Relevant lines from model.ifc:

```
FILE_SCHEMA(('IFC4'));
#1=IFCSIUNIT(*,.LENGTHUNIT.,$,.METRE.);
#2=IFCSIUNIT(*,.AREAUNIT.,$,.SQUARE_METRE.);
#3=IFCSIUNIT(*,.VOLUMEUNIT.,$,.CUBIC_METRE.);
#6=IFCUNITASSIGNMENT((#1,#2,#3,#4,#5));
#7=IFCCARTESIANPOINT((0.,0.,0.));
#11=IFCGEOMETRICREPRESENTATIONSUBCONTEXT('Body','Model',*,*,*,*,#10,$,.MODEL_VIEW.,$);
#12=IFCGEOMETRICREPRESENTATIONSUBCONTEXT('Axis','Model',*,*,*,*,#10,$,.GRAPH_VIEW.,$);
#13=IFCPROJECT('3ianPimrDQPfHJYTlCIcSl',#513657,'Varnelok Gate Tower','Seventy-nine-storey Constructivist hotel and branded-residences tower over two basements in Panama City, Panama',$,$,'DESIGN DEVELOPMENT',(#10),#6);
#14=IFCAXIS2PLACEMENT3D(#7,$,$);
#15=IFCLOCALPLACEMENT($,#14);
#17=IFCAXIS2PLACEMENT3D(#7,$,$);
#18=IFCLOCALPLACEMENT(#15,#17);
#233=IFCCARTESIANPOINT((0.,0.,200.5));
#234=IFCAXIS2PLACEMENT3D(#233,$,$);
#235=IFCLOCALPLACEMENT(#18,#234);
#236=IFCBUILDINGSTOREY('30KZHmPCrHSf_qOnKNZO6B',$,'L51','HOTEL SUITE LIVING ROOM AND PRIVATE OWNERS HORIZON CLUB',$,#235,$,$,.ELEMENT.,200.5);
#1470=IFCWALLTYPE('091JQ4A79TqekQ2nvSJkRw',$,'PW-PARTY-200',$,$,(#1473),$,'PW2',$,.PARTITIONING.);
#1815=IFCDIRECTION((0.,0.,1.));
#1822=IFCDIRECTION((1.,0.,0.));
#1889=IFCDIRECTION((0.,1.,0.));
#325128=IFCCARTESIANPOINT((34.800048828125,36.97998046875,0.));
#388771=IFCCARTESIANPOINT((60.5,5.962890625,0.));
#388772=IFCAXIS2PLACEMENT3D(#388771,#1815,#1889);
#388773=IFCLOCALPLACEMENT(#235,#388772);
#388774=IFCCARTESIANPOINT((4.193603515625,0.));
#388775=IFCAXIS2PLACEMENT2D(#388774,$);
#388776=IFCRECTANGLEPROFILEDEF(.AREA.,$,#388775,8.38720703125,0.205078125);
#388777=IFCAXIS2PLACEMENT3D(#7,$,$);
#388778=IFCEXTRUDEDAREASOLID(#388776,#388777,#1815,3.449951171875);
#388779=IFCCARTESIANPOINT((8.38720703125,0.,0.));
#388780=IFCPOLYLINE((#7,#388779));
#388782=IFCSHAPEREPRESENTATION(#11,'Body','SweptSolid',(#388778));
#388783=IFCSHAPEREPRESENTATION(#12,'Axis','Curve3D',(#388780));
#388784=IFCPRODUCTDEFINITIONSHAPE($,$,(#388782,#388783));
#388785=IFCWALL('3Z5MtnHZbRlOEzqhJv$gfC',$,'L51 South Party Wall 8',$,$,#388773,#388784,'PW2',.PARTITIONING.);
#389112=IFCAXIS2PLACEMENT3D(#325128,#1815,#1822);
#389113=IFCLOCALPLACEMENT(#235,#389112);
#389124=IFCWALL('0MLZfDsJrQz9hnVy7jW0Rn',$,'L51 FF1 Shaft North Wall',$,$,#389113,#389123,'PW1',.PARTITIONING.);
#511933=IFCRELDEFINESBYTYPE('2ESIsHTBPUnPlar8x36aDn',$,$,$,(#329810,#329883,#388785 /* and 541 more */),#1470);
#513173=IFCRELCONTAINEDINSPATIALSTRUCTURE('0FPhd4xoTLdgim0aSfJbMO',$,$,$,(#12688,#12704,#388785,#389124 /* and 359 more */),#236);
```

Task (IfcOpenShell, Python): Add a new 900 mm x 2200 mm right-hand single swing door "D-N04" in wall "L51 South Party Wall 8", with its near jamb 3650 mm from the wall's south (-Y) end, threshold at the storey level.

```python
import numpy as np
import ifcopenshell
import ifcopenshell.api.feature
import ifcopenshell.api.geometry
import ifcopenshell.api.root
import ifcopenshell.api.spatial
import ifcopenshell.geom
import ifcopenshell.util.element
import ifcopenshell.util.placement
import ifcopenshell.util.representation
import ifcopenshell.util.shape
import ifcopenshell.util.unit

model = ifcopenshell.open("model.ifc")
unit_scale = ifcopenshell.util.unit.calculate_unit_scale(model)
settings = ifcopenshell.geom.settings()


def volume(element):
    """Net volume in cubic metres, openings subtracted."""
    shape = ifcopenshell.geom.create_shape(settings, element)
    return ifcopenshell.util.shape.get_volume(shape.geometry)


wall = model.by_id(388785)
storey = ifcopenshell.util.element.get_container(wall, ifc_class="IfcBuildingStorey")
context = ifcopenshell.util.representation.get_context(model, "Model", "Body", "MODEL_VIEW")
before = volume(wall)

width, height, from_end, sill = 0.9, 2.2, 3.65, 0.0  # metres

# The wall runs along its own X axis, and the end named is its -X end.
wall_shape = ifcopenshell.geom.create_shape(settings, wall)
x, y, z = ifcopenshell.util.shape.get_vertices(wall_shape.geometry).T
start = x.min() + from_end
face, thickness = float(y.min()), float(y.max() - y.min())
wall_matrix = ifcopenshell.util.placement.get_local_placement(wall.ObjectPlacement)
level = ifcopenshell.util.placement.get_local_placement(storey.ObjectPlacement)[2, 3]


def in_wall(x, y):
    """Placement at x, y metres in the wall's axes, at sill height."""
    matrix = wall_matrix.copy()
    matrix[:, 3] = wall_matrix @ np.array([x / unit_scale, y / unit_scale, 0.0, 1.0])
    matrix[2, 3] = level + sill / unit_scale
    return matrix


# Opening: a box that overshoots both wall faces by 50 mm.
opening = ifcopenshell.api.root.create_entity(model, ifc_class="IfcOpeningElement", predefined_type="OPENING")
box = ifcopenshell.api.geometry.add_wall_representation(
    model, context=context, length=width, height=height, thickness=thickness + 0.1
)
ifcopenshell.api.geometry.assign_representation(model, product=opening, representation=box)
ifcopenshell.api.geometry.edit_object_placement(model, product=opening, matrix=in_wall(start, face - 0.05), is_si=False)
ifcopenshell.api.feature.add_feature(model, feature=opening, element=wall)

door = ifcopenshell.api.root.create_entity(model, ifc_class="IfcDoor", name="D-N04", predefined_type="DOOR")
door.OverallWidth, door.OverallHeight = width / unit_scale, height / unit_scale
door.OperationType = "SINGLE_SWING_RIGHT"
body = ifcopenshell.api.geometry.add_door_representation(
    model,
    context=context,
    overall_width=door.OverallWidth,
    overall_height=door.OverallHeight,
    operation_type="SINGLE_SWING_RIGHT",
    lining_properties={"LiningDepth": thickness / unit_scale, "ThresholdDepth": thickness / unit_scale},
)
ifcopenshell.api.geometry.assign_representation(model, product=door, representation=body)
ifcopenshell.api.spatial.assign_container(model, products=[door], relating_structure=storey)
ifcopenshell.api.feature.add_filling(model, opening=opening, element=door)

# The lining spans the wall, so the door starts at the wall face.
ifcopenshell.api.geometry.edit_object_placement(model, product=door, matrix=in_wall(start, face), is_si=False)

after = volume(wall)

print(f"wall volume {before:.3f} -> {after:.3f} m3")

model.write("model-out.ifc")
```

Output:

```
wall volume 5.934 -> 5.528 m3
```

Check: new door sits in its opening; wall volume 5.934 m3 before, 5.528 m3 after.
